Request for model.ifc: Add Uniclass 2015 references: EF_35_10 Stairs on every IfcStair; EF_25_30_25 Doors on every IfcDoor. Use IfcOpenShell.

First a look at what the model holds.

```python
import ifcopenshell

model = ifcopenshell.open("model.ifc")
print(model.schema)
print("classifications:", [c.Name for c in model.by_type("IfcClassification")])
for ifc_class in ("IfcDoor", "IfcRoof", "IfcStair", "IfcWall", "IfcWindow"):
    print(ifc_class, len(model.by_type(ifc_class)))
```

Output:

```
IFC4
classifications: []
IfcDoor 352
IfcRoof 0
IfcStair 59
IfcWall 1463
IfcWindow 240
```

```python
import ifcopenshell
import ifcopenshell.api.classification

model = ifcopenshell.open("model.ifc")

system = ifcopenshell.api.classification.add_classification(model, classification="Uniclass 2015")

codes = {
    "IfcStair": ("EF_35_10", "Stairs"),
    "IfcDoor": ("EF_25_30_25", "Doors"),
}
for ifc_class, (code, name) in codes.items():
    products = model.by_type(ifc_class)
    ifcopenshell.api.classification.add_reference(
        model, products=products, classification=system, identification=code, name=name
    )
    print(code, len(products))

model.write("model_updated.ifc")
```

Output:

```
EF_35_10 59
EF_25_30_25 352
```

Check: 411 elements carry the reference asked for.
